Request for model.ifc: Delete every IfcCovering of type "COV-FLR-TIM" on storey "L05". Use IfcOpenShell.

First a look at what the model holds.

```python
import ifcopenshell
import ifcopenshell.util.element

model = ifcopenshell.open("model.ifc")
print(model.schema)
storey = next(s for s in model.by_type("IfcBuildingStorey") if s.Name == "L05")
coverings = [e for e in ifcopenshell.util.element.get_decomposition(storey) if e.is_a("IfcCovering")]
seen = {}
for e in coverings:
    element_type = ifcopenshell.util.element.get_type(e)
    name = element_type.Name if element_type not in (None, e) else None
    seen[name] = seen.get(name, 0) + 1
for name, count in sorted(seen.items(), key=str):
    print(count, "x", name)
```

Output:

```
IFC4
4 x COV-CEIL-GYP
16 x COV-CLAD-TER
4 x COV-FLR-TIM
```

```python
import ifcopenshell
import ifcopenshell.api.root
import ifcopenshell.util.element

model = ifcopenshell.open("model.ifc")

storey = next(s for s in model.by_type("IfcBuildingStorey") if s.Name == "L05")
coverings = [e for e in ifcopenshell.util.element.get_decomposition(storey) if e.is_a("IfcCovering")]
targets = [e for e in coverings if (t := ifcopenshell.util.element.get_type(e)) not in (None, e) and t.Name == "COV-FLR-TIM"]

for e in targets:
    ifcopenshell.api.root.remove_product(model, product=e)
print(len(targets), "removed")

model.write("model-out.ifc")
```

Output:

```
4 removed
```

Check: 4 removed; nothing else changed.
